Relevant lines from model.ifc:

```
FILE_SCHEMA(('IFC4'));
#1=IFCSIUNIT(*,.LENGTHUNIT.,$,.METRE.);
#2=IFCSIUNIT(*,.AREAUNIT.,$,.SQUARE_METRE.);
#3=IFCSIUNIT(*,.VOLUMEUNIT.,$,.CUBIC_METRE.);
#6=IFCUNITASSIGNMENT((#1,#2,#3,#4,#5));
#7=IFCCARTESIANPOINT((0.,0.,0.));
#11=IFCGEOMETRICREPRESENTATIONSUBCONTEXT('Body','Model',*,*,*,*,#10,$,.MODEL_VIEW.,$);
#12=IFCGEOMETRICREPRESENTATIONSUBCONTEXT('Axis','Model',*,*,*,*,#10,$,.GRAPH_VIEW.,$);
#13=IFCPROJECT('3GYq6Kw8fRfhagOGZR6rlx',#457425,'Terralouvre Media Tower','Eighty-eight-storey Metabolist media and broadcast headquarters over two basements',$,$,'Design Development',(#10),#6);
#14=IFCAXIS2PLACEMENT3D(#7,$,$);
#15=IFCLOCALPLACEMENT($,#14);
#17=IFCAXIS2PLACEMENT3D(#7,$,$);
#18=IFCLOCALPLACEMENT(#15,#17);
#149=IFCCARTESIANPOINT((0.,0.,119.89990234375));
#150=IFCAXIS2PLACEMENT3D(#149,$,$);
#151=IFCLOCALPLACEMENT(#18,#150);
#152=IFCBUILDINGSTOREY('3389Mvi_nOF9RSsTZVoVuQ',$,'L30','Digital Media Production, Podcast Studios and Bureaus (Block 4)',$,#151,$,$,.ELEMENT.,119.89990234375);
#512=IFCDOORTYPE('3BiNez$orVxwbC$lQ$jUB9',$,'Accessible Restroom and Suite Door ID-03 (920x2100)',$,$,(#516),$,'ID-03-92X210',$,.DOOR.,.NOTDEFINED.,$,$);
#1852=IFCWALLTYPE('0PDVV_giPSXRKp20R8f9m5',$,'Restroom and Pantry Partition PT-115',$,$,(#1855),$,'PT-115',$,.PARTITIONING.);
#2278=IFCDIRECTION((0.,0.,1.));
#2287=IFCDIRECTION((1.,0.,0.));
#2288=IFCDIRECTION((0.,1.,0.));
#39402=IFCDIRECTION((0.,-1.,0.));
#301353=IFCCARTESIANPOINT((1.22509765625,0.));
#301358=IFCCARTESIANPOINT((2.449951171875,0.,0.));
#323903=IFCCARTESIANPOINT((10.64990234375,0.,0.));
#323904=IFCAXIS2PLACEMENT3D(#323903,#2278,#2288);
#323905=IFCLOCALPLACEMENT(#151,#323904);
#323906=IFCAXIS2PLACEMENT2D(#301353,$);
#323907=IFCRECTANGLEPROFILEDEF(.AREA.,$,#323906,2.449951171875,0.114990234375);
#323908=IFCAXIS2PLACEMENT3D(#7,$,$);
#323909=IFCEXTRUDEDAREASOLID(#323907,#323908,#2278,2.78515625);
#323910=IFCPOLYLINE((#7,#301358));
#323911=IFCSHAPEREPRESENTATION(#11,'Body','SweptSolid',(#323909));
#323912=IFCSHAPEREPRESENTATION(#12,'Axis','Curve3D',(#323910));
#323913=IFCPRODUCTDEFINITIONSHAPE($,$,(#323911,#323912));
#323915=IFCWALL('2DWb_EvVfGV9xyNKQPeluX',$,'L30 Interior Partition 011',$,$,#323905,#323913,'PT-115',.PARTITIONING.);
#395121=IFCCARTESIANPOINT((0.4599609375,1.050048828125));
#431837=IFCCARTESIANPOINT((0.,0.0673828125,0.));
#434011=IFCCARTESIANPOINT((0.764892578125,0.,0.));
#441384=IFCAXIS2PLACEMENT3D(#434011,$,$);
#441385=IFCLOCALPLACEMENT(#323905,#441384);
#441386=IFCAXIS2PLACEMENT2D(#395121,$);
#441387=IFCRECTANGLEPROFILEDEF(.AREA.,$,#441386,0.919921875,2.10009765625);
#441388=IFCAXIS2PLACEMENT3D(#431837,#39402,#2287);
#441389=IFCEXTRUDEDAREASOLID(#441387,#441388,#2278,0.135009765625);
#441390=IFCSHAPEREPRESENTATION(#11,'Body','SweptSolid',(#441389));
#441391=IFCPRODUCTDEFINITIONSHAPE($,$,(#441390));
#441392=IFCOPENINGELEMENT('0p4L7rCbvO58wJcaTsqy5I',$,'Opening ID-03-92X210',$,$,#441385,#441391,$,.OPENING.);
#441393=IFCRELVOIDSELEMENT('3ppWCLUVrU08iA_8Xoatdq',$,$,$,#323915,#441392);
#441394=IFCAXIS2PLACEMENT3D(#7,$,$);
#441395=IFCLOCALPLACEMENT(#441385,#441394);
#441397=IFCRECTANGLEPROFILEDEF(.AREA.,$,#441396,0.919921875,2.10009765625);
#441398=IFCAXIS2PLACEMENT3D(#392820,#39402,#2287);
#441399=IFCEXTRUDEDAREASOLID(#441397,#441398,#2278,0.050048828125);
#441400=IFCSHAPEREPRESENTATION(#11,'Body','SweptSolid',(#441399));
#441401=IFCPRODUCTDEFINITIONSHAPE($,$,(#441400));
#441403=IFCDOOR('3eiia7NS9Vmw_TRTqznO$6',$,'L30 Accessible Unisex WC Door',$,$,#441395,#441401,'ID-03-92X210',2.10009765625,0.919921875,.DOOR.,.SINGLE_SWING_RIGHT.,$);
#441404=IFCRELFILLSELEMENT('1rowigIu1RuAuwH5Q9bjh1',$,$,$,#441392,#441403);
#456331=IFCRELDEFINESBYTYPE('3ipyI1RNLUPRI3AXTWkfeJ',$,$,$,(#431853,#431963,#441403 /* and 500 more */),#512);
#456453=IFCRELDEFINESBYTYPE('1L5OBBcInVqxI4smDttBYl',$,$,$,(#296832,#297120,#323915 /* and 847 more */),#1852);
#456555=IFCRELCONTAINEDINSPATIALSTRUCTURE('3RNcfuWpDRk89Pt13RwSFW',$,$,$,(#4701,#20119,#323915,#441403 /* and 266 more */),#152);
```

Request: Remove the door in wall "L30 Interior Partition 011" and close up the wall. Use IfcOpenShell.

```python
import ifcopenshell
import ifcopenshell.api.feature
import ifcopenshell.api.root
import ifcopenshell.geom
import ifcopenshell.util.shape

model = ifcopenshell.open("model.ifc")
settings = ifcopenshell.geom.settings()


def volume(element):
    """Net volume in cubic metres, openings subtracted."""
    shape = ifcopenshell.geom.create_shape(settings, element)
    return ifcopenshell.util.shape.get_volume(shape.geometry)


door = model.by_guid("3eiia7NS9Vmw_TRTqznO$6")
opening = door.FillsVoids[0].RelatingOpeningElement
wall = opening.VoidsElements[0].RelatingBuildingElement
before = volume(wall)

ifcopenshell.api.root.remove_product(model, product=door)
ifcopenshell.api.feature.remove_feature(model, feature=opening)

after = volume(wall)

print(f"wall volume {before:.3f} -> {after:.3f} m3")

model.write("model-out.ifc")
```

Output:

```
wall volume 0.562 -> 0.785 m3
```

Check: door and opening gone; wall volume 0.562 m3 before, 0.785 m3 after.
